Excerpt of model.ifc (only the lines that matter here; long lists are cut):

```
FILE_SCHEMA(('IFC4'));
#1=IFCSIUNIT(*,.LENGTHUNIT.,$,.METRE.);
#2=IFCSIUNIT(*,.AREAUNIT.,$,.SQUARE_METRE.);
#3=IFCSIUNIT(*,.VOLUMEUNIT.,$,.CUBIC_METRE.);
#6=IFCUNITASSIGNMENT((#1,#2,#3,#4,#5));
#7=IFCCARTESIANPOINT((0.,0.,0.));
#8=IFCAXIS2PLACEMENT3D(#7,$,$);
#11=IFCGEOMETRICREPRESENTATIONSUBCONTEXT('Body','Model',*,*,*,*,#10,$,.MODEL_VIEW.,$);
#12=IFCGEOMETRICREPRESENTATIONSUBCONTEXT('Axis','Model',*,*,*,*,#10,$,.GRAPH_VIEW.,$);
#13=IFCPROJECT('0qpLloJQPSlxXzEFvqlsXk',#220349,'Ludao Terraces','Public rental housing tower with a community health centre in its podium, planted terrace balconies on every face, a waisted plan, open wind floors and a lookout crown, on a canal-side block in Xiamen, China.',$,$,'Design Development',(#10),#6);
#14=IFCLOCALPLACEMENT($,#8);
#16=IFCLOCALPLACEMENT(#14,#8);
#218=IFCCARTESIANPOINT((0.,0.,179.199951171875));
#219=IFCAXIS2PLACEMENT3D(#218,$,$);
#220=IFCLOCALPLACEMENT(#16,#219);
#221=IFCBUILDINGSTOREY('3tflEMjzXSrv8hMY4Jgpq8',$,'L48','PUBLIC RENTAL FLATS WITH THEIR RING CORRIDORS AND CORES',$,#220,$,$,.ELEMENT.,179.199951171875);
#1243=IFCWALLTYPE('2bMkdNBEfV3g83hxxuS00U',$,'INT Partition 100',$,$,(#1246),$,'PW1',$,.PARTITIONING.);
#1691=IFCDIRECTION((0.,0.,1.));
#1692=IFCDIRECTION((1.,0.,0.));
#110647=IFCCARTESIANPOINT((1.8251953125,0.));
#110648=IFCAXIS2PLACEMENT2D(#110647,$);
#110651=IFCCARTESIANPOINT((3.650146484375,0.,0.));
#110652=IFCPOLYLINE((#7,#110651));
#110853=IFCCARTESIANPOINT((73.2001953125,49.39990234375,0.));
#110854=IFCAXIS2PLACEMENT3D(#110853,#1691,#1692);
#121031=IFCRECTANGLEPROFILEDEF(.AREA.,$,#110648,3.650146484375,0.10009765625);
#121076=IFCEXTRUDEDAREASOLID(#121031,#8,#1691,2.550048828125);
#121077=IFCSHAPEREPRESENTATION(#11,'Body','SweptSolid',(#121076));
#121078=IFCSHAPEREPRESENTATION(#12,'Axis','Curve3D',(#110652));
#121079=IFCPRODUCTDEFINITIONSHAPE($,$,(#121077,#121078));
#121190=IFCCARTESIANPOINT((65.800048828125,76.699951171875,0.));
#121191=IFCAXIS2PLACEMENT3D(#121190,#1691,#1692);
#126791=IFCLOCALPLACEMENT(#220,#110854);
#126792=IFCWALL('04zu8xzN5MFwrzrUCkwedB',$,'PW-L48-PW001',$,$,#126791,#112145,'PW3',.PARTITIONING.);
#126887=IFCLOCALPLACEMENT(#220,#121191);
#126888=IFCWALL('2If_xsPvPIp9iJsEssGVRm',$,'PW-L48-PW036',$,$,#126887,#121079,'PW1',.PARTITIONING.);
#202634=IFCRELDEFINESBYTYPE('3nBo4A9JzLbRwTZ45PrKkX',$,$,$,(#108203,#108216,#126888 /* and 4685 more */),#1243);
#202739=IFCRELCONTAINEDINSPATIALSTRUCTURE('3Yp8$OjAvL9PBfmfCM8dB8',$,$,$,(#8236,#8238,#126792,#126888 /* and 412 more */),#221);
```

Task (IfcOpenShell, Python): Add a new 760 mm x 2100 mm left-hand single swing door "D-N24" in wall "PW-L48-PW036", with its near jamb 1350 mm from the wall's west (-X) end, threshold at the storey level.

```python
import numpy as np
import ifcopenshell
import ifcopenshell.api.feature
import ifcopenshell.api.geometry
import ifcopenshell.api.root
import ifcopenshell.api.spatial
import ifcopenshell.geom
import ifcopenshell.util.element
import ifcopenshell.util.placement
import ifcopenshell.util.representation
import ifcopenshell.util.shape
import ifcopenshell.util.unit

model = ifcopenshell.open("model.ifc")
unit_scale = ifcopenshell.util.unit.calculate_unit_scale(model)
settings = ifcopenshell.geom.settings()


def volume(element):
    """Net volume in cubic metres, openings subtracted."""
    shape = ifcopenshell.geom.create_shape(settings, element)
    return ifcopenshell.util.shape.get_volume(shape.geometry)


wall = model.by_guid("2If_xsPvPIp9iJsEssGVRm")
storey = ifcopenshell.util.element.get_container(wall, ifc_class="IfcBuildingStorey")
context = ifcopenshell.util.representation.get_context(model, "Model", "Body", "MODEL_VIEW")
before = volume(wall)

width, height, from_end, sill = 0.76, 2.1, 1.35, 0.0  # metres

# The wall runs along its own X axis, and the end named is its -X end.
wall_shape = ifcopenshell.geom.create_shape(settings, wall)
x, y, z = ifcopenshell.util.shape.get_vertices(wall_shape.geometry).T
start = x.min() + from_end
face, thickness = float(y.min()), float(y.max() - y.min())
wall_matrix = ifcopenshell.util.placement.get_local_placement(wall.ObjectPlacement)
level = ifcopenshell.util.placement.get_local_placement(storey.ObjectPlacement)[2, 3]


def in_wall(x, y):
    """Placement at x, y metres in the wall's axes, at sill height."""
    matrix = wall_matrix.copy()
    matrix[:, 3] = wall_matrix @ np.array([x / unit_scale, y / unit_scale, 0.0, 1.0])
    matrix[2, 3] = level + sill / unit_scale
    return matrix


# Opening: a box that overshoots both wall faces by 50 mm.
opening = ifcopenshell.api.root.create_entity(model, ifc_class="IfcOpeningElement", predefined_type="OPENING")
box = ifcopenshell.api.geometry.add_wall_representation(
    model, context=context, length=width, height=height, thickness=thickness + 0.1
)
ifcopenshell.api.geometry.assign_representation(model, product=opening, representation=box)
ifcopenshell.api.geometry.edit_object_placement(model, product=opening, matrix=in_wall(start, face - 0.05), is_si=False)
ifcopenshell.api.feature.add_feature(model, feature=opening, element=wall)

door = ifcopenshell.api.root.create_entity(model, ifc_class="IfcDoor", name="D-N24", predefined_type="DOOR")
door.OverallWidth, door.OverallHeight = width / unit_scale, height / unit_scale
door.OperationType = "SINGLE_SWING_LEFT"
body = ifcopenshell.api.geometry.add_door_representation(
    model,
    context=context,
    overall_width=door.OverallWidth,
    overall_height=door.OverallHeight,
    operation_type="SINGLE_SWING_LEFT",
    lining_properties={"LiningDepth": thickness / unit_scale, "ThresholdDepth": thickness / unit_scale},
)
ifcopenshell.api.geometry.assign_representation(model, product=door, representation=body)
ifcopenshell.api.spatial.assign_container(model, products=[door], relating_structure=storey)
ifcopenshell.api.feature.add_filling(model, opening=opening, element=door)

# The lining spans the wall, so the door starts at the wall face.
ifcopenshell.api.geometry.edit_object_placement(model, product=door, matrix=in_wall(start, face), is_si=False)

after = volume(wall)

print(f"wall volume {before:.3f} -> {after:.3f} m3")

model.write("model_v2.ifc")
```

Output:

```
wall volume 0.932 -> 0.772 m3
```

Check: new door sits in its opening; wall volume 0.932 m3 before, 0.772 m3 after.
